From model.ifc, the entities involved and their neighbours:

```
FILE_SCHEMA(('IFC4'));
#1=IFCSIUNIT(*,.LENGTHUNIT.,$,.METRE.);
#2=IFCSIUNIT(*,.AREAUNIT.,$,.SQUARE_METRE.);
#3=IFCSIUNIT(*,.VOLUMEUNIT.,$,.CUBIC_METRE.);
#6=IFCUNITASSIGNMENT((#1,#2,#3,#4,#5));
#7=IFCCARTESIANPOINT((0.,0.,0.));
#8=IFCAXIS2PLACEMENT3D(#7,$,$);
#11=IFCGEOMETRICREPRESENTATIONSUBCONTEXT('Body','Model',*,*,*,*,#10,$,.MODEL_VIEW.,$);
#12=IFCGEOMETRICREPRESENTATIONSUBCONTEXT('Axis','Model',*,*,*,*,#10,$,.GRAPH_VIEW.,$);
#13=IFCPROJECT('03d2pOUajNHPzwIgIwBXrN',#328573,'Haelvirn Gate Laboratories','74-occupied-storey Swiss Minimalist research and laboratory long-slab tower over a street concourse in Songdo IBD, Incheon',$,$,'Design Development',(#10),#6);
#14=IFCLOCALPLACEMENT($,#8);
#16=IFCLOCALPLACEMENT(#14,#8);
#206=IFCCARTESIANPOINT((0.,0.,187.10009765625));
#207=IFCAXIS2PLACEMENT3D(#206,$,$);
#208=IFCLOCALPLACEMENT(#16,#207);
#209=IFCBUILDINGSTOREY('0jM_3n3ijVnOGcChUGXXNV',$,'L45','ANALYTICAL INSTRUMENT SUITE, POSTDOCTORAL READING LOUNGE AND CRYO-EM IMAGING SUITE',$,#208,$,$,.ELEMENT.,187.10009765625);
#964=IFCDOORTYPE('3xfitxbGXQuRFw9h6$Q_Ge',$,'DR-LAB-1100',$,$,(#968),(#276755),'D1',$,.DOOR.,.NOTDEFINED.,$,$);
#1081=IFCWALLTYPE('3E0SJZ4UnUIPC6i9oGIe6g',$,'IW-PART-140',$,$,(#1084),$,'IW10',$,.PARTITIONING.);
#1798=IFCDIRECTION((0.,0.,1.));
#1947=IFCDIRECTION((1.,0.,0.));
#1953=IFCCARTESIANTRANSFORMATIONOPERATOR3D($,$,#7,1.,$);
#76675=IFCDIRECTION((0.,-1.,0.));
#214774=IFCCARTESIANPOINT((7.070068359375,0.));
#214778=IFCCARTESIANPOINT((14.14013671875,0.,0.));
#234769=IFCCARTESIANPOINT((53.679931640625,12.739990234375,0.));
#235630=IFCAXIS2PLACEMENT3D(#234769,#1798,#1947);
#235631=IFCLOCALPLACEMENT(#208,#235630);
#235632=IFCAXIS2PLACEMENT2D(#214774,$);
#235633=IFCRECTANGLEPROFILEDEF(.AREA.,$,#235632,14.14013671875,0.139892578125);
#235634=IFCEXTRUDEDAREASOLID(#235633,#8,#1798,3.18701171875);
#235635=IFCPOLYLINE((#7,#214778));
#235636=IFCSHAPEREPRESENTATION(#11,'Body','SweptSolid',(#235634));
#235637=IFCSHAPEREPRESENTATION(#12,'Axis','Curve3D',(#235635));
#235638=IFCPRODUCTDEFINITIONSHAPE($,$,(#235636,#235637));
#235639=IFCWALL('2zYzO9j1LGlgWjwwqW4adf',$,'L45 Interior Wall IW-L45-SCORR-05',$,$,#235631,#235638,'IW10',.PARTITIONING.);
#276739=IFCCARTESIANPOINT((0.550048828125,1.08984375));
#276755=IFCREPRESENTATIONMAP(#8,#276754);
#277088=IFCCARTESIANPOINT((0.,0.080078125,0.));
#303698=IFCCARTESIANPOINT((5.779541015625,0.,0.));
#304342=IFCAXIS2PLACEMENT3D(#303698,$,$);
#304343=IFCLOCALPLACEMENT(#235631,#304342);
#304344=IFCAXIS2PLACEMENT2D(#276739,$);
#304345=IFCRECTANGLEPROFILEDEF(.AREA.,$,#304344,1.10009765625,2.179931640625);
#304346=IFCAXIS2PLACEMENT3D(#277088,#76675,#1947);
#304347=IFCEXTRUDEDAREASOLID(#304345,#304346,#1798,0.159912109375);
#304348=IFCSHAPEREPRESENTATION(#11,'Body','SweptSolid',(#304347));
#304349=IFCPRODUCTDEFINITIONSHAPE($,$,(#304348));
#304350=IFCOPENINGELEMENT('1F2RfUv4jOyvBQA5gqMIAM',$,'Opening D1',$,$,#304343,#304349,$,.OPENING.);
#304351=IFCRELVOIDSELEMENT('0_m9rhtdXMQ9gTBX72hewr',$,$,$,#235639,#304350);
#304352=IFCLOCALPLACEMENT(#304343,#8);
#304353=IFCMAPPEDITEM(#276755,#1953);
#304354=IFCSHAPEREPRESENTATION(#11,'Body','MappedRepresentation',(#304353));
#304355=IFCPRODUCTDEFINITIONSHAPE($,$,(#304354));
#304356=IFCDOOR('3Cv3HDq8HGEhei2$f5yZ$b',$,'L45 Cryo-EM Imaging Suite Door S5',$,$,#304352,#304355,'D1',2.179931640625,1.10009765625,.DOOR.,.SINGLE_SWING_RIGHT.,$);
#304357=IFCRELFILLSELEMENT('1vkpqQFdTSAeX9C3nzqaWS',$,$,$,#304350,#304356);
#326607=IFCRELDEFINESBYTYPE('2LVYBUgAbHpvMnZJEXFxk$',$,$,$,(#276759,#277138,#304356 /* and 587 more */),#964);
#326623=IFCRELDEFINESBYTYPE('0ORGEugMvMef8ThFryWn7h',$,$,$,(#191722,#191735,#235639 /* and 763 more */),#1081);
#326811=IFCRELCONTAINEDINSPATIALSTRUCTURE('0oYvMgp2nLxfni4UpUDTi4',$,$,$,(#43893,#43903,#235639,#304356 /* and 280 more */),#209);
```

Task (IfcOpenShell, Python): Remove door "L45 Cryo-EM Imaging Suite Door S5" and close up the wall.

```python
import ifcopenshell
import ifcopenshell.api.feature
import ifcopenshell.api.root
import ifcopenshell.geom
import ifcopenshell.util.shape

model = ifcopenshell.open("model.ifc")
settings = ifcopenshell.geom.settings()


def volume(element):
    """Net volume in cubic metres, openings subtracted."""
    shape = ifcopenshell.geom.create_shape(settings, element)
    return ifcopenshell.util.shape.get_volume(shape.geometry)


door = model.by_guid("3Cv3HDq8HGEhei2$f5yZ$b")
opening = door.FillsVoids[0].RelatingOpeningElement
wall = opening.VoidsElements[0].RelatingBuildingElement
before = volume(wall)

ifcopenshell.api.root.remove_product(model, product=door)
ifcopenshell.api.feature.remove_feature(model, feature=opening)

after = volume(wall)

print(f"wall volume {before:.3f} -> {after:.3f} m3")

model.write("model_rev.ifc")
```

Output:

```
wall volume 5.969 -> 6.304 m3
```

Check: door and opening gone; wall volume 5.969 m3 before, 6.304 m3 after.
